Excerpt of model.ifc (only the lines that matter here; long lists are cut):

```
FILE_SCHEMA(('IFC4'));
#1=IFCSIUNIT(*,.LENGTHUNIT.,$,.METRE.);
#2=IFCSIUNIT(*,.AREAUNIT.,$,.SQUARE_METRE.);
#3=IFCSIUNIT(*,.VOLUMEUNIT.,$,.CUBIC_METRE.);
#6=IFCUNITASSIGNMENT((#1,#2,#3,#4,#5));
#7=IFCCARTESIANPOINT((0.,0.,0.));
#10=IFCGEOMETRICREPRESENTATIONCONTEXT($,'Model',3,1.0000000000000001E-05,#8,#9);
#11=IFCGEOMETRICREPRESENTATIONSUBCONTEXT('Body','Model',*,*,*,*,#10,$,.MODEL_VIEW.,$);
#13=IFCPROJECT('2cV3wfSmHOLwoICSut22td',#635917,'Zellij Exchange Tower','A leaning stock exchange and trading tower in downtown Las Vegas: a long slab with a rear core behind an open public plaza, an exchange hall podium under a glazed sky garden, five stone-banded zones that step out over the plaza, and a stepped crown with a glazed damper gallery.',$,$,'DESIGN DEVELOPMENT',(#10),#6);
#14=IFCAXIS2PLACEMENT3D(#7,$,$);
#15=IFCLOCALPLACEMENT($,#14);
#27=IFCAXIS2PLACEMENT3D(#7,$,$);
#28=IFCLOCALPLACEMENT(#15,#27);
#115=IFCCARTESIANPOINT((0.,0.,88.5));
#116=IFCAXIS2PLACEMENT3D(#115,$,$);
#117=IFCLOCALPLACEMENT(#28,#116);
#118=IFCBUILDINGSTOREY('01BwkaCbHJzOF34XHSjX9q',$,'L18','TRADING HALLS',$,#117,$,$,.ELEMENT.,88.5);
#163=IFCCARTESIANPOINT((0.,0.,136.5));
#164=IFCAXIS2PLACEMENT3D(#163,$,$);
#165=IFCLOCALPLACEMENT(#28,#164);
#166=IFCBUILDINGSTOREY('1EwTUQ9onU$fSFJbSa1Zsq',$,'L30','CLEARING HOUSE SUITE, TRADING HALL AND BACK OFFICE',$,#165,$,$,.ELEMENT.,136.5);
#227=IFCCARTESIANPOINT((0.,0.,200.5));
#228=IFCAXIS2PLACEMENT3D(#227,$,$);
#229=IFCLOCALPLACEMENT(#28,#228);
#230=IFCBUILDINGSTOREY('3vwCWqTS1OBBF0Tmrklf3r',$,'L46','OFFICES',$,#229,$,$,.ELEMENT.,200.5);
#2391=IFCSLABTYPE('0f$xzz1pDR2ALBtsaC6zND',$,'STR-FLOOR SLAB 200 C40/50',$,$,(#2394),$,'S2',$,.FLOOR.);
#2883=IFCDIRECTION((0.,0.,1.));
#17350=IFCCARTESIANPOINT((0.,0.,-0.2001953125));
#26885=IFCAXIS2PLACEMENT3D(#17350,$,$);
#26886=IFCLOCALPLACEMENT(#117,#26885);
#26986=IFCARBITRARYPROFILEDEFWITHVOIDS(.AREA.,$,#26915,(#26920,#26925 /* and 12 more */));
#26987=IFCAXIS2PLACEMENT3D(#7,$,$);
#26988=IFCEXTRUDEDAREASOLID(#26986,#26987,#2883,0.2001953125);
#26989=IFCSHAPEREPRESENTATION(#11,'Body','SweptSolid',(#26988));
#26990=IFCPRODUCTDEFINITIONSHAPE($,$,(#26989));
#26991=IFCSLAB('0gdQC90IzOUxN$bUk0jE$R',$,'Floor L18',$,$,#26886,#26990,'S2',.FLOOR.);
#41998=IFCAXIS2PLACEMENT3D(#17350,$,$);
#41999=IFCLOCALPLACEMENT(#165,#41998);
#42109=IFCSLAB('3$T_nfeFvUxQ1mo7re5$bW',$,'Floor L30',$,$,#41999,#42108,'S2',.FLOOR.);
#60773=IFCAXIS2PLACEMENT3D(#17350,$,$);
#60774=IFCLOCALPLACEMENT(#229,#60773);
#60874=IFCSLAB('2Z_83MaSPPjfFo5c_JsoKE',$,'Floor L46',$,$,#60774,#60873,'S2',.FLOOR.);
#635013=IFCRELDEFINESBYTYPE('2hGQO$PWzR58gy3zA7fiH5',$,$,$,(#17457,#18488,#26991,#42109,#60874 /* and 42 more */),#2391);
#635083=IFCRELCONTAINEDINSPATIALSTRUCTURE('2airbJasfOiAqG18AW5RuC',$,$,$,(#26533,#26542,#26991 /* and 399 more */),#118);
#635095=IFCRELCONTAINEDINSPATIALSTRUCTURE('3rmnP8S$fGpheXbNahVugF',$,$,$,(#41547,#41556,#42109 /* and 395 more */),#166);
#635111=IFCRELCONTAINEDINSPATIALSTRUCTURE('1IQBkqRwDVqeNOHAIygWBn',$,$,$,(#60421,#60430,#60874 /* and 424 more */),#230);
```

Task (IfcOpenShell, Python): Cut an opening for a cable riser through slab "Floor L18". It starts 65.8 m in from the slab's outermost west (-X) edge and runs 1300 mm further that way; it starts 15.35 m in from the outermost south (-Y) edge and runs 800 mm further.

```python
import numpy as np
import ifcopenshell
import ifcopenshell.api.feature
import ifcopenshell.api.geometry
import ifcopenshell.api.root
import ifcopenshell.geom
import ifcopenshell.util.placement
import ifcopenshell.util.representation
import ifcopenshell.util.shape
import ifcopenshell.util.unit

model = ifcopenshell.open("model.ifc")
unit_scale = ifcopenshell.util.unit.calculate_unit_scale(model)
settings = ifcopenshell.geom.settings()


def volume(element):
    """Net volume in cubic metres, openings subtracted."""
    shape = ifcopenshell.geom.create_shape(settings, element)
    return ifcopenshell.util.shape.get_volume(shape.geometry)


slab = model.by_guid("0gdQC90IzOUxN$bUk0jE$R")
before = volume(slab)

# Extent in the slab's own axes, in metres. The edges named are its -X and -Y sides.
slab_shape = ifcopenshell.geom.create_shape(settings, slab)
vertices = ifcopenshell.util.shape.get_vertices(slab_shape.geometry)
x_min, y_min, bottom = vertices.min(axis=0)
top = vertices[:, 2].max()

opening = ifcopenshell.api.root.create_entity(model, ifc_class="IfcOpeningElement", name="Cable riser opening", predefined_type="OPENING")
context = ifcopenshell.util.representation.get_context(model, "Model", "Body", "MODEL_VIEW")
width, depth = 1.3, 0.8
outline = [(0.0, 0.0), (width, 0.0), (width, depth), (0.0, depth), (0.0, 0.0)]
# Overshoot both faces by 50 mm so the cut is clean.
shape = ifcopenshell.api.geometry.add_slab_representation(
    model, context=context, depth=top - bottom + 0.1, polyline=outline
)
ifcopenshell.api.geometry.assign_representation(model, product=opening, representation=shape)

matrix = ifcopenshell.util.placement.get_local_placement(slab.ObjectPlacement)
matrix[:, 3] = matrix @ np.append(np.array([x_min + 65.8, y_min + 15.35, bottom - 0.05]) / unit_scale, 1.0)
ifcopenshell.api.geometry.edit_object_placement(model, product=opening, matrix=matrix, is_si=False)
ifcopenshell.api.feature.add_feature(model, feature=opening, element=slab)

after = volume(slab)

print(f"slab volume {before:.3f} -> {after:.3f} m3")

model.write("model_rev.ifc")
```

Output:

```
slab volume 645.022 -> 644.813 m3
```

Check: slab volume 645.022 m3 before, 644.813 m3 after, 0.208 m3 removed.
